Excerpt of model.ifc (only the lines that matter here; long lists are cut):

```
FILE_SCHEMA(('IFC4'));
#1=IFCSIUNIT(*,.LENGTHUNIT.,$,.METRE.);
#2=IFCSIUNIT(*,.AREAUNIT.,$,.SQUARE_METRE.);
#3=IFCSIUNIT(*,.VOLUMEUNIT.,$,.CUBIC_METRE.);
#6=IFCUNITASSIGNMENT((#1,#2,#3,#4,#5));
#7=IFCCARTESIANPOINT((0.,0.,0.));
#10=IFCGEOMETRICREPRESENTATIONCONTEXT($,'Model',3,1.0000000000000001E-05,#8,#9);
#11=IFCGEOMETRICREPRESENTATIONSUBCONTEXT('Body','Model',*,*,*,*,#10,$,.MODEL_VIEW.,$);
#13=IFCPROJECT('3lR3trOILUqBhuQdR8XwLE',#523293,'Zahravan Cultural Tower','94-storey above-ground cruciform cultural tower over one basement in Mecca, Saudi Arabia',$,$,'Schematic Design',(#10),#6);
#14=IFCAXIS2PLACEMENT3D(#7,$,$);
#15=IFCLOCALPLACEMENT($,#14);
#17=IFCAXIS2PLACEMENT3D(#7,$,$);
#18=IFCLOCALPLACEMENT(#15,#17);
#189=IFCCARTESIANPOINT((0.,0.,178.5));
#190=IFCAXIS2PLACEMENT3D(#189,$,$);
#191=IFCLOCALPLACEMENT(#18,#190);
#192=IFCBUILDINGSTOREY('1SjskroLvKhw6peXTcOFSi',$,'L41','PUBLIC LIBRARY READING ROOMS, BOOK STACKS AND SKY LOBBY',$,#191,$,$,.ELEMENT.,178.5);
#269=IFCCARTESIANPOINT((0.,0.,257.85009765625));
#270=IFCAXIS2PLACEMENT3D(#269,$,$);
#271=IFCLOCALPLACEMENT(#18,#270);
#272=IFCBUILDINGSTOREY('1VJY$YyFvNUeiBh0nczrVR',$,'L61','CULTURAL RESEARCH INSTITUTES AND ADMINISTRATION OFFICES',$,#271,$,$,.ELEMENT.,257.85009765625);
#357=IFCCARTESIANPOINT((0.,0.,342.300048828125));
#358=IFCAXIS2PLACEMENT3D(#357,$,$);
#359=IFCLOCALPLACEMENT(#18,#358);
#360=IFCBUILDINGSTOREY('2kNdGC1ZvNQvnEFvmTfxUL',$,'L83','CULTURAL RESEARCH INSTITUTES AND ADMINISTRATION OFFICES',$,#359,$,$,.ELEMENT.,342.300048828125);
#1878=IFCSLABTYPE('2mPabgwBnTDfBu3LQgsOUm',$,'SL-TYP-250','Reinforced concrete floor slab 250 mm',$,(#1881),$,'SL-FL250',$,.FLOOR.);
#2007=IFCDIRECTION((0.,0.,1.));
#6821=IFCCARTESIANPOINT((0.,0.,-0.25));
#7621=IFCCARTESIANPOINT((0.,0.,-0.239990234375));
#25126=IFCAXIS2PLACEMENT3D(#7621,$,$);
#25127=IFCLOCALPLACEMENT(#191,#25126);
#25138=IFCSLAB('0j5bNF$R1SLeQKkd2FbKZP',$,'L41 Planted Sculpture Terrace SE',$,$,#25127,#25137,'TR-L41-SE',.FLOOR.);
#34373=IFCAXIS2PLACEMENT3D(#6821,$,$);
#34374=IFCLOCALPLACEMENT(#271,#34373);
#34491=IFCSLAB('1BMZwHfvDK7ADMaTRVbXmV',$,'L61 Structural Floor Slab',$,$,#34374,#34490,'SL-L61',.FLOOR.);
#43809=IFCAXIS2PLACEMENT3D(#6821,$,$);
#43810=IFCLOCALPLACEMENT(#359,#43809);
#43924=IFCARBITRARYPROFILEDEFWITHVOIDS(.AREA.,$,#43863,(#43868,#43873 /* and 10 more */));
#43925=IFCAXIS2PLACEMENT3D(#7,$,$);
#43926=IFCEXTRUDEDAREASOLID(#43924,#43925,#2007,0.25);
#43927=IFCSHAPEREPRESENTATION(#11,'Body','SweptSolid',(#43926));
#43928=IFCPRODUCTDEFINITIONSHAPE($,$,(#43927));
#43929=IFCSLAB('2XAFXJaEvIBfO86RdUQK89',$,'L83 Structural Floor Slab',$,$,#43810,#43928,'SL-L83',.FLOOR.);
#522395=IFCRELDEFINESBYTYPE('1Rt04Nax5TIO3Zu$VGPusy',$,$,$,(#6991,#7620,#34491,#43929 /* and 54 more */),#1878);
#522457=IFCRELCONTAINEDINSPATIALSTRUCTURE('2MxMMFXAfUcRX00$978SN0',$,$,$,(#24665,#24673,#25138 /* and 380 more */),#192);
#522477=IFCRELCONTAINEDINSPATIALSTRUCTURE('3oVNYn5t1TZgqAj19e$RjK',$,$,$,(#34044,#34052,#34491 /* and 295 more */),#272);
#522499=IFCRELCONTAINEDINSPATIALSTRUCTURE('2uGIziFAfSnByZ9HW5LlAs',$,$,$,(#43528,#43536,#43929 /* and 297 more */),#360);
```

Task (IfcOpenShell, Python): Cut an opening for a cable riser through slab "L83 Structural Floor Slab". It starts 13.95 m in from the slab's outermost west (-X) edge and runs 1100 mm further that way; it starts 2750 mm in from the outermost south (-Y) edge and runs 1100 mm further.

```python
import numpy as np
import ifcopenshell
import ifcopenshell.api.feature
import ifcopenshell.api.geometry
import ifcopenshell.api.root
import ifcopenshell.geom
import ifcopenshell.util.placement
import ifcopenshell.util.representation
import ifcopenshell.util.shape
import ifcopenshell.util.unit

model = ifcopenshell.open("model.ifc")
unit_scale = ifcopenshell.util.unit.calculate_unit_scale(model)
settings = ifcopenshell.geom.settings()


def volume(element):
    """Net volume in cubic metres, openings subtracted."""
    shape = ifcopenshell.geom.create_shape(settings, element)
    return ifcopenshell.util.shape.get_volume(shape.geometry)


slab = model.by_guid("2XAFXJaEvIBfO86RdUQK89")
before = volume(slab)

# Extent in the slab's own axes, in metres. The edges named are its -X and -Y sides.
slab_shape = ifcopenshell.geom.create_shape(settings, slab)
vertices = ifcopenshell.util.shape.get_vertices(slab_shape.geometry)
x_min, y_min, bottom = vertices.min(axis=0)
top = vertices[:, 2].max()

opening = ifcopenshell.api.root.create_entity(model, ifc_class="IfcOpeningElement", name="Cable riser opening", predefined_type="OPENING")
context = ifcopenshell.util.representation.get_context(model, "Model", "Body", "MODEL_VIEW")
width, depth = 1.1, 1.1
outline = [(0.0, 0.0), (width, 0.0), (width, depth), (0.0, depth), (0.0, 0.0)]
# Overshoot both faces by 50 mm so the cut is clean.
shape = ifcopenshell.api.geometry.add_slab_representation(
    model, context=context, depth=top - bottom + 0.1, polyline=outline
)
ifcopenshell.api.geometry.assign_representation(model, product=opening, representation=shape)

matrix = ifcopenshell.util.placement.get_local_placement(slab.ObjectPlacement)
matrix[:, 3] = matrix @ np.append(np.array([x_min + 13.95, y_min + 2.75, bottom - 0.05]) / unit_scale, 1.0)
ifcopenshell.api.geometry.edit_object_placement(model, product=opening, matrix=matrix, is_si=False)
ifcopenshell.api.feature.add_feature(model, feature=opening, element=slab)

after = volume(slab)

print(f"slab volume {before:.3f} -> {after:.3f} m3")

model.write("model-out.ifc")
```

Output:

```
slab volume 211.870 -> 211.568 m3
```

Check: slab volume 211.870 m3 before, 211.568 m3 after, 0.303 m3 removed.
